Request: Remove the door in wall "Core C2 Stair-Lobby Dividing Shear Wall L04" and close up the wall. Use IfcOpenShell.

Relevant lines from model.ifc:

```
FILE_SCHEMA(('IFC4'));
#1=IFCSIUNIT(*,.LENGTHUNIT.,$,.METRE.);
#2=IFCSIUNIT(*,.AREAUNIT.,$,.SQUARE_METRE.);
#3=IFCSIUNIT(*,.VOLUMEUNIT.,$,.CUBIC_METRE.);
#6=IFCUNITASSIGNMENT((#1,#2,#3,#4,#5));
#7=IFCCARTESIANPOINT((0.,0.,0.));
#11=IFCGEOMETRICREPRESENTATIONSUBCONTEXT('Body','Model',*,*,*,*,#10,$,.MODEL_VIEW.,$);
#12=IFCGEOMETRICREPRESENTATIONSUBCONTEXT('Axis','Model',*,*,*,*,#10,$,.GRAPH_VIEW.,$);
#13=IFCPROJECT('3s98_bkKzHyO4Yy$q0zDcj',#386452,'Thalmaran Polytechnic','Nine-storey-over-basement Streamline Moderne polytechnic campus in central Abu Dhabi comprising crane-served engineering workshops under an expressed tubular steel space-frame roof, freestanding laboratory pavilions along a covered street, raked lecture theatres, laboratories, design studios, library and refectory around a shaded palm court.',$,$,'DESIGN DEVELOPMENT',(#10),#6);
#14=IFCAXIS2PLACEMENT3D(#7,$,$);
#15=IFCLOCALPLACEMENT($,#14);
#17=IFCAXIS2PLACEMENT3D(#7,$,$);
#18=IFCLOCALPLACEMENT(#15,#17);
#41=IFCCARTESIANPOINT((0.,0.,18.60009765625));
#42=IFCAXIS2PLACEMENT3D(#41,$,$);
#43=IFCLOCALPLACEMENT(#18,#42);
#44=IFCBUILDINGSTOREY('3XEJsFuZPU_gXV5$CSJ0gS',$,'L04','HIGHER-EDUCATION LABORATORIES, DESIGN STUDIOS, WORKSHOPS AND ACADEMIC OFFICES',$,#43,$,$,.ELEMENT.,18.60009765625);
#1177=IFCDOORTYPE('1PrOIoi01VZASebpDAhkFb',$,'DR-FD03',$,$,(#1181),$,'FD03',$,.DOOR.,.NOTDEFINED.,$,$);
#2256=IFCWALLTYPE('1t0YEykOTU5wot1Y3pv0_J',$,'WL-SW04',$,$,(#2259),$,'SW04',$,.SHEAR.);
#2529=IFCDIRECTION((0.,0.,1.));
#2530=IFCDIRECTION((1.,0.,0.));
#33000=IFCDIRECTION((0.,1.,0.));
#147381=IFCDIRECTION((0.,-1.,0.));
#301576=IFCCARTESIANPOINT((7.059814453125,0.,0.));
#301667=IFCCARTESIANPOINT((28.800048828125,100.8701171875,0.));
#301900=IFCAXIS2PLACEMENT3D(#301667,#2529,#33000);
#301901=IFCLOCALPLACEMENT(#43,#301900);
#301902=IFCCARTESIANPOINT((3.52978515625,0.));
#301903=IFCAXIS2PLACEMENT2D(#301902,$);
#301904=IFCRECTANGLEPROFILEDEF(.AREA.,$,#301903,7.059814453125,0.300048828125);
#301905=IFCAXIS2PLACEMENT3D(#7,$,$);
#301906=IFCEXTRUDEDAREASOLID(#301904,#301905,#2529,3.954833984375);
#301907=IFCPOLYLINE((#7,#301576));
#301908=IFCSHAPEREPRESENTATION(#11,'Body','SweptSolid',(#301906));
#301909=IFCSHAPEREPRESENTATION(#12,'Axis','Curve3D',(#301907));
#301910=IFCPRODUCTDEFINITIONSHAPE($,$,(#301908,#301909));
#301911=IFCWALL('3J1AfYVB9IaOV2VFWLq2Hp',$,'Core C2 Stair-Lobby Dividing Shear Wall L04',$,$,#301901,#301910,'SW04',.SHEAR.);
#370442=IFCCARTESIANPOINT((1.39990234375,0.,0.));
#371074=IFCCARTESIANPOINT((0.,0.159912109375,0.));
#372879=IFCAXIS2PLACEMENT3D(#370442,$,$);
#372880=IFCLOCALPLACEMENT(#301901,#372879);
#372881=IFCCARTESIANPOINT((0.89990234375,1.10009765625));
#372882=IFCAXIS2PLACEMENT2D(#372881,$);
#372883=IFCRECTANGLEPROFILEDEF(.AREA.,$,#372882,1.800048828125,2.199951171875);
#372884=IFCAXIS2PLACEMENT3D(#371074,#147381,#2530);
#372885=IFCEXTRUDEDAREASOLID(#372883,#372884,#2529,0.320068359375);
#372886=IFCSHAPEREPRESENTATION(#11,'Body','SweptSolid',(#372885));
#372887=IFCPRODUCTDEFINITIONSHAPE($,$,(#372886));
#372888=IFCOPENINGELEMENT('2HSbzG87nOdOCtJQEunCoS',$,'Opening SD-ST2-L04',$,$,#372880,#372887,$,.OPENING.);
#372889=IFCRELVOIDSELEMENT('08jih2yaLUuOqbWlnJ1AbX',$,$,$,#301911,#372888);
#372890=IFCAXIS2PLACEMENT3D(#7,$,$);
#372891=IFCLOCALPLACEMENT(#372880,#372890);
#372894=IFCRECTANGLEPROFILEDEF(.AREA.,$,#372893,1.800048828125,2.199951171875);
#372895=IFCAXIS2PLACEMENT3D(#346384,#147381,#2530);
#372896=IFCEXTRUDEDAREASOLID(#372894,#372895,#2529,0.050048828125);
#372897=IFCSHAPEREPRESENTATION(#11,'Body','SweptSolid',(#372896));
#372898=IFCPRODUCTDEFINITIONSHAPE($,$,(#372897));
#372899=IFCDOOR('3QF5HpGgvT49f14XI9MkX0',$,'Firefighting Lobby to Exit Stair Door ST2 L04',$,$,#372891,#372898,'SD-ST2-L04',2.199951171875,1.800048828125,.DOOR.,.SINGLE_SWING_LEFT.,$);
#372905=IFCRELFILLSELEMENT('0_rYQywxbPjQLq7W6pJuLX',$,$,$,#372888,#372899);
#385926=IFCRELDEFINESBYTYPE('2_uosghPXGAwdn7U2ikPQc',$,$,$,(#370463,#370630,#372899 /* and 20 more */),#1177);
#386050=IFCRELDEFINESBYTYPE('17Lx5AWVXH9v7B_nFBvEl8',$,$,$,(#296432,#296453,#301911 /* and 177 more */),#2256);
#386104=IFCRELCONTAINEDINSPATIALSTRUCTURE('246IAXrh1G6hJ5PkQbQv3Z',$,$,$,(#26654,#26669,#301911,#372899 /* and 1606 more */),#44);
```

```python
import ifcopenshell
import ifcopenshell.api.feature
import ifcopenshell.api.root
import ifcopenshell.geom
import ifcopenshell.util.shape

model = ifcopenshell.open("model.ifc")
settings = ifcopenshell.geom.settings()


def volume(element):
    """Net volume in cubic metres, openings subtracted."""
    shape = ifcopenshell.geom.create_shape(settings, element)
    return ifcopenshell.util.shape.get_volume(shape.geometry)


door = model.by_id(372899)
opening = door.FillsVoids[0].RelatingOpeningElement
wall = opening.VoidsElements[0].RelatingBuildingElement
before = volume(wall)

ifcopenshell.api.root.remove_product(model, product=door)
ifcopenshell.api.feature.remove_feature(model, feature=opening)

after = volume(wall)

print(f"wall volume {before:.3f} -> {after:.3f} m3")

model.write("model_v2.ifc")
```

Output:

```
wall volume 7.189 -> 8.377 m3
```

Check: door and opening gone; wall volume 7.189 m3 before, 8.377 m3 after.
